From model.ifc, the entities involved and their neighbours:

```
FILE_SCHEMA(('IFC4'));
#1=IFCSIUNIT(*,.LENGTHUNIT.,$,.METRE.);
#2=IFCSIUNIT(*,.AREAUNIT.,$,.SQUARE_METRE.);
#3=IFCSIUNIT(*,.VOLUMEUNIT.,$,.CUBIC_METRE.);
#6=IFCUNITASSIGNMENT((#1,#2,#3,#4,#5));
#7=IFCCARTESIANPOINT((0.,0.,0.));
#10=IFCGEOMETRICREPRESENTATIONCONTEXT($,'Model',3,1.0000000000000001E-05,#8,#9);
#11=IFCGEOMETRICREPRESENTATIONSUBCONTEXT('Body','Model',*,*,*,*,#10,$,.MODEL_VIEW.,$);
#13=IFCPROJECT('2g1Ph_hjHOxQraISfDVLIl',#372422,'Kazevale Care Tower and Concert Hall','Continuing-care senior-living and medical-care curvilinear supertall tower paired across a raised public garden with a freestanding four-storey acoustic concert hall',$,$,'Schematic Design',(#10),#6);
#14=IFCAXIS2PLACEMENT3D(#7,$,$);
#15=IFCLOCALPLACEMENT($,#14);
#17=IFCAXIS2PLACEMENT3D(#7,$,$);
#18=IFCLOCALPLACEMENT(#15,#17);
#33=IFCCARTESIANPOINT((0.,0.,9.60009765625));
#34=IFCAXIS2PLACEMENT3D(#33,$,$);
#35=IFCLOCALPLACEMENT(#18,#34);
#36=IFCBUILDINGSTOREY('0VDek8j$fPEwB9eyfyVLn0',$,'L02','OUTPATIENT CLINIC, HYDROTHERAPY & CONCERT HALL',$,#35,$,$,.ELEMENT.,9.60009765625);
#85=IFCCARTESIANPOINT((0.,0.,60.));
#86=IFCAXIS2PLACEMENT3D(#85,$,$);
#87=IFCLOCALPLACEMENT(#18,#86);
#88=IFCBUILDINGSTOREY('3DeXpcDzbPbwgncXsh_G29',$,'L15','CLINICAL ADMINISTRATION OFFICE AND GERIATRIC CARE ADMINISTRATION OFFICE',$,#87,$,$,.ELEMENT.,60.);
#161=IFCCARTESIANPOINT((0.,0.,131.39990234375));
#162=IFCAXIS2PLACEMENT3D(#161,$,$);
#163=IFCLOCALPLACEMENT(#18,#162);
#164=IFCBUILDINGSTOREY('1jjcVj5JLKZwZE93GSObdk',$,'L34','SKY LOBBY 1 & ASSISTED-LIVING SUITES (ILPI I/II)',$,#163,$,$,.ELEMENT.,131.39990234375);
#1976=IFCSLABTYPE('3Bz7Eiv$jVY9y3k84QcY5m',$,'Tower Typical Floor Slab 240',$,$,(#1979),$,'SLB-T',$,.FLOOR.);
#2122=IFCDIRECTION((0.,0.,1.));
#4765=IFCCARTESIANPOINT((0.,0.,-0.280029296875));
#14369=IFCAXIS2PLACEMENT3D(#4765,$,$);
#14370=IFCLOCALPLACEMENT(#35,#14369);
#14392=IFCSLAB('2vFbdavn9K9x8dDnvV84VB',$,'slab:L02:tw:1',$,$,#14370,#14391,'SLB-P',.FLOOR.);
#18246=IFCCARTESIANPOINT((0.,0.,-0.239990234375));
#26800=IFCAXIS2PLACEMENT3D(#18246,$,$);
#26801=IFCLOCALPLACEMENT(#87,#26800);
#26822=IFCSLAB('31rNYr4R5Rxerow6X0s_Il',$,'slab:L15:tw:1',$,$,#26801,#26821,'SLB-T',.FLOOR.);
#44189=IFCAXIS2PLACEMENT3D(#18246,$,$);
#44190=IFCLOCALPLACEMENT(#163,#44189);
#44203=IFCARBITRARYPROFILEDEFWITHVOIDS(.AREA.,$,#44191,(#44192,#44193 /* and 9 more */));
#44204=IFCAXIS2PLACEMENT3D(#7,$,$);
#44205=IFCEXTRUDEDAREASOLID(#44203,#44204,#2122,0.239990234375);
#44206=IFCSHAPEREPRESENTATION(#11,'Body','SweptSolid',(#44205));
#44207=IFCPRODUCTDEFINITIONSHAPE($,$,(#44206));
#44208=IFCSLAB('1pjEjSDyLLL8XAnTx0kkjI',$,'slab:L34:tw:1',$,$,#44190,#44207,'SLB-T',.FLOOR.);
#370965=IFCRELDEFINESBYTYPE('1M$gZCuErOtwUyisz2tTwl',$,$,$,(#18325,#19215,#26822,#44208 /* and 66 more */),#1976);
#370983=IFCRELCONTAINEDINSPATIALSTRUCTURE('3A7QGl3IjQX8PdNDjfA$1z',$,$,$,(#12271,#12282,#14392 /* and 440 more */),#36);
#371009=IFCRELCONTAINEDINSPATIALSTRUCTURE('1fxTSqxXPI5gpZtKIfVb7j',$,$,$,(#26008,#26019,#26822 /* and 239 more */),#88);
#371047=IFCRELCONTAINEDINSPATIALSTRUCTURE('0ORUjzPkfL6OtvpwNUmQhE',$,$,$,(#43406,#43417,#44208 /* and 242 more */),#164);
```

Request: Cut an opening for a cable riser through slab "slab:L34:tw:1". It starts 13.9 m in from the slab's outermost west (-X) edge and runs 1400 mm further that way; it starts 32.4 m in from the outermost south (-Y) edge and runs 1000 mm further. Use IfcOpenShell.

```python
import numpy as np
import ifcopenshell
import ifcopenshell.api.feature
import ifcopenshell.api.geometry
import ifcopenshell.api.root
import ifcopenshell.geom
import ifcopenshell.util.placement
import ifcopenshell.util.representation
import ifcopenshell.util.shape
import ifcopenshell.util.unit

model = ifcopenshell.open("model.ifc")
unit_scale = ifcopenshell.util.unit.calculate_unit_scale(model)
settings = ifcopenshell.geom.settings()


def volume(element):
    """Net volume in cubic metres, openings subtracted."""
    shape = ifcopenshell.geom.create_shape(settings, element)
    return ifcopenshell.util.shape.get_volume(shape.geometry)


slab = model.by_guid("1pjEjSDyLLL8XAnTx0kkjI")
before = volume(slab)

# Extent in the slab's own axes, in metres. The edges named are its -X and -Y sides.
slab_shape = ifcopenshell.geom.create_shape(settings, slab)
vertices = ifcopenshell.util.shape.get_vertices(slab_shape.geometry)
x_min, y_min, bottom = vertices.min(axis=0)
top = vertices[:, 2].max()

opening = ifcopenshell.api.root.create_entity(model, ifc_class="IfcOpeningElement", name="Cable riser opening", predefined_type="OPENING")
context = ifcopenshell.util.representation.get_context(model, "Model", "Body", "MODEL_VIEW")
width, depth = 1.4, 1
outline = [(0.0, 0.0), (width, 0.0), (width, depth), (0.0, depth), (0.0, 0.0)]
# Overshoot both faces by 50 mm so the cut is clean.
shape = ifcopenshell.api.geometry.add_slab_representation(
    model, context=context, depth=top - bottom + 0.1, polyline=outline
)
ifcopenshell.api.geometry.assign_representation(model, product=opening, representation=shape)

matrix = ifcopenshell.util.placement.get_local_placement(slab.ObjectPlacement)
matrix[:, 3] = matrix @ np.append(np.array([x_min + 13.9, y_min + 32.4, bottom - 0.05]) / unit_scale, 1.0)
ifcopenshell.api.geometry.edit_object_placement(model, product=opening, matrix=matrix, is_si=False)
ifcopenshell.api.feature.add_feature(model, feature=opening, element=slab)

after = volume(slab)

print(f"slab volume {before:.3f} -> {after:.3f} m3")

model.write("model_rev.ifc")
```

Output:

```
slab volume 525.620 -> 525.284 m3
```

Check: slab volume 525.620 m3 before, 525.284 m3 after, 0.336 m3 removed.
